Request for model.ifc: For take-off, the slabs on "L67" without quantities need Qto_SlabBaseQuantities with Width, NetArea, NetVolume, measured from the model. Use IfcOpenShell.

First a look at what the model holds.

```python
import ifcopenshell
import ifcopenshell.util.element
import ifcopenshell.util.unit

model = ifcopenshell.open("model.ifc")
print(model.schema)
for unit_type in ("LENGTHUNIT", "AREAUNIT", "VOLUMEUNIT"):
    print(unit_type, ifcopenshell.util.unit.calculate_unit_scale(model, unit_type))
storey = next(s for s in model.by_type("IfcBuildingStorey") if s.Name == "L67")
slabs = [e for e in ifcopenshell.util.element.get_decomposition(storey) if e.is_a("IfcSlab")]
for e in sorted(slabs, key=lambda e: e.id()):
    print(e.id(), e.is_a(), e.Name, list(ifcopenshell.util.element.get_psets(e, qtos_only=True)), sep=" | ")
```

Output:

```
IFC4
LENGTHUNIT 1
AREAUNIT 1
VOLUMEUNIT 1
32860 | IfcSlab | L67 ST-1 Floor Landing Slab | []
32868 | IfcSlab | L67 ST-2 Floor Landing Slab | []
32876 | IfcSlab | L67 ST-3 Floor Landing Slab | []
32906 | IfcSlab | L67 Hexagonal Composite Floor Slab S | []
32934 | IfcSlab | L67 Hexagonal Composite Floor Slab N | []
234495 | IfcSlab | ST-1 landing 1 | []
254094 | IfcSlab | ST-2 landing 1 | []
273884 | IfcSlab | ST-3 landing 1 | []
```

```python
import ifcopenshell
import ifcopenshell.api.pset
import ifcopenshell.geom
import ifcopenshell.util.element
import ifcopenshell.util.shape
import ifcopenshell.util.unit

model = ifcopenshell.open("model.ifc")
unit_scale = ifcopenshell.util.unit.calculate_unit_scale(model)
area_scale = ifcopenshell.util.unit.calculate_unit_scale(model, "AREAUNIT")
volume_scale = ifcopenshell.util.unit.calculate_unit_scale(model, "VOLUMEUNIT")
settings = ifcopenshell.geom.settings()

storey = next(s for s in model.by_type("IfcBuildingStorey") if s.Name == "L67")
slabs = [e for e in ifcopenshell.util.element.get_decomposition(storey) if e.is_a("IfcSlab")]

for e in sorted(slabs, key=lambda e: e.id()):
    if ifcopenshell.util.element.get_psets(e, qtos_only=True, should_inherit=False):
        continue
    # Geometry comes back in metres, in the element's own axes.
    shape = ifcopenshell.geom.create_shape(settings, e)
    values = {
        "Width": ifcopenshell.util.shape.get_z(shape.geometry) / unit_scale,
        "NetArea": ifcopenshell.util.shape.get_footprint_area(shape.geometry) / area_scale,
        "NetVolume": ifcopenshell.util.shape.get_volume(shape.geometry) / volume_scale,
    }
    qto = ifcopenshell.api.pset.add_qto(model, product=e, name="Qto_SlabBaseQuantities")
    ifcopenshell.api.pset.edit_qto(model, qto=qto, properties=values)
    print(e.id(), {k: round(v, 3) for k, v in values.items()})

model.write("model_edited.ifc")
```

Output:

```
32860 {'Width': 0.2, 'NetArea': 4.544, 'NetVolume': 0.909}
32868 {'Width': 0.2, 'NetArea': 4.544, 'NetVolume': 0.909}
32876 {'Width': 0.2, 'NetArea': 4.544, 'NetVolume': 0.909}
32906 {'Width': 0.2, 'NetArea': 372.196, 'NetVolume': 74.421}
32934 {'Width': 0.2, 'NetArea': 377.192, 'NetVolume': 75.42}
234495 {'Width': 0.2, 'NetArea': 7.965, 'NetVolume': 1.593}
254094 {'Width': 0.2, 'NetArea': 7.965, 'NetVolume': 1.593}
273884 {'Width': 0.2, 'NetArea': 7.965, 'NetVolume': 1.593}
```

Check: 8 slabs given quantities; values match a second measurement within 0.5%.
